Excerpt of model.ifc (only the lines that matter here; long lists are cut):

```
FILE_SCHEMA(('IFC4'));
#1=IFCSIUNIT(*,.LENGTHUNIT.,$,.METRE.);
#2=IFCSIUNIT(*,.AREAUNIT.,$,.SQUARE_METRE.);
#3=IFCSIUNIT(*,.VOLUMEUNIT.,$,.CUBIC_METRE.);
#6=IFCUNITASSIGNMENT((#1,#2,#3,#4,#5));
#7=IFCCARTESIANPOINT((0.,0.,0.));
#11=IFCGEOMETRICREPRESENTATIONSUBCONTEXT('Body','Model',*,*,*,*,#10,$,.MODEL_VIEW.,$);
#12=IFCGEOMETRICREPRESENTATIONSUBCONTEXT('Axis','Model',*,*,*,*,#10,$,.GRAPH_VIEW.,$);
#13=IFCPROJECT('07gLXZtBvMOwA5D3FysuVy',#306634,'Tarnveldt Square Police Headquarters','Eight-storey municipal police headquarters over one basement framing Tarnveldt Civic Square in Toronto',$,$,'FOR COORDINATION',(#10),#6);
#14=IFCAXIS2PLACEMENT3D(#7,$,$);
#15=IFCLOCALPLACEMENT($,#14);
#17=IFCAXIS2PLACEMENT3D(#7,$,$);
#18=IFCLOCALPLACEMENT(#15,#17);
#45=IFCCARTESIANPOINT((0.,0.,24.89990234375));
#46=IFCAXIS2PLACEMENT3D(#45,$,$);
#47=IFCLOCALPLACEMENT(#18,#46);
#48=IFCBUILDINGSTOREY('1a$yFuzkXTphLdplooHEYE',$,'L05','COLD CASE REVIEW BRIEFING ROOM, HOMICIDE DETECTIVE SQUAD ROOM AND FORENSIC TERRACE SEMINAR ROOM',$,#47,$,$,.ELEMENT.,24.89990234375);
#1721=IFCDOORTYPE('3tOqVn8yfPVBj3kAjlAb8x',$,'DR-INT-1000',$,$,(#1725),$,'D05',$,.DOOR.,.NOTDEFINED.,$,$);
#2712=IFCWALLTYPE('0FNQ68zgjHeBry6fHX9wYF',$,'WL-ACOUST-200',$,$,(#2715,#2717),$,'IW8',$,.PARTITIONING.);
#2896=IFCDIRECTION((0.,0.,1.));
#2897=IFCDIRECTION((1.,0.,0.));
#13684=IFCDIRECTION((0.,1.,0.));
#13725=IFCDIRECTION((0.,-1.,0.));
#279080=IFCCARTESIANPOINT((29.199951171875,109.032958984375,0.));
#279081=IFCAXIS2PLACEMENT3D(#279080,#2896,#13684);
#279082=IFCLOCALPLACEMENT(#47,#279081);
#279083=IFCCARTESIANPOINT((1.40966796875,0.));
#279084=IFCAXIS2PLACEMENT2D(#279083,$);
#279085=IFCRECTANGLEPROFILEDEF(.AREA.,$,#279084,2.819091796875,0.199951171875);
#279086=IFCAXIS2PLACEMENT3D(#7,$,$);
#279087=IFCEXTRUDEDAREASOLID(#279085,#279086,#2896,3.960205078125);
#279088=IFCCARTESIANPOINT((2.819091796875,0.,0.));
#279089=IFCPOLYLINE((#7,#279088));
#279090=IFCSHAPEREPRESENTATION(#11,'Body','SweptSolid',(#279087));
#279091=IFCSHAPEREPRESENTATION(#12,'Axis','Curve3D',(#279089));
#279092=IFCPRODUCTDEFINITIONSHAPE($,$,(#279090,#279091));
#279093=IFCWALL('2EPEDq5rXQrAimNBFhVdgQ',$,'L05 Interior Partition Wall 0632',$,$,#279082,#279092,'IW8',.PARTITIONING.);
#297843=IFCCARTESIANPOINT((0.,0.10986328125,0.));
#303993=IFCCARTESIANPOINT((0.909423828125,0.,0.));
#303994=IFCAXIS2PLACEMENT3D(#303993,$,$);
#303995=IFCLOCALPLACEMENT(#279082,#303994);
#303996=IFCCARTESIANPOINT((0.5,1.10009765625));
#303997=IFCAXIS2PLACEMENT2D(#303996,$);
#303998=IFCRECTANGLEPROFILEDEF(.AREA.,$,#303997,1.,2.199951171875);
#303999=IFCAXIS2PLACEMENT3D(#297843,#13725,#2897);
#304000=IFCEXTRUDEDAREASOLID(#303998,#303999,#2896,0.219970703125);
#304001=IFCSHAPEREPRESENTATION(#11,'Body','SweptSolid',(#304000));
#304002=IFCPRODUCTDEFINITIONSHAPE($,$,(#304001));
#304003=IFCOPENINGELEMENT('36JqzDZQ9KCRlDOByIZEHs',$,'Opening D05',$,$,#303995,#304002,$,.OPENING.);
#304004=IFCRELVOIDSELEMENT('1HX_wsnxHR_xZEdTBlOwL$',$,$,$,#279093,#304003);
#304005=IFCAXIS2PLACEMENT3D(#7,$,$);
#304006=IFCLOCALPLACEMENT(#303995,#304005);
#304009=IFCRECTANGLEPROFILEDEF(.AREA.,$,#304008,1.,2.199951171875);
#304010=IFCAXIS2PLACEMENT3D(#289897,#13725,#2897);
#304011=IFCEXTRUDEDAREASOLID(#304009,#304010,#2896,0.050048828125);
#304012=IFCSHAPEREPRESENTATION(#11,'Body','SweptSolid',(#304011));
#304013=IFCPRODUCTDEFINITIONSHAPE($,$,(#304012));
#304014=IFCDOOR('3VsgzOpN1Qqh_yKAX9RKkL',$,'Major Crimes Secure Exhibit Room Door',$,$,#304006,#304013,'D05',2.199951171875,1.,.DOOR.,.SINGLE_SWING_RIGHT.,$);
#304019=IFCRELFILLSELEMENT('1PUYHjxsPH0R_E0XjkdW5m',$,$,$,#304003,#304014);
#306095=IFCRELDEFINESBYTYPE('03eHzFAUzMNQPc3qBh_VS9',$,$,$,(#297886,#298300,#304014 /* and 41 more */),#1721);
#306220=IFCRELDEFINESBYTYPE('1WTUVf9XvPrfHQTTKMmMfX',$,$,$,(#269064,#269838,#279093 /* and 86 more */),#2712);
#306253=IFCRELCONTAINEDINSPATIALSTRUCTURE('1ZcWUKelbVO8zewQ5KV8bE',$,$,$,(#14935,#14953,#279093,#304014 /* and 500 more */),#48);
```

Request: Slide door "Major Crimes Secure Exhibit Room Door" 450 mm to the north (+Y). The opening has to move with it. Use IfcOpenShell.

```python
import ifcopenshell
import ifcopenshell.api.geometry
import ifcopenshell.util.placement
import ifcopenshell.util.unit

model = ifcopenshell.open("model.ifc")
unit_scale = ifcopenshell.util.unit.calculate_unit_scale(model)

door = model.by_id(304014)
opening = door.FillsVoids[0].RelatingOpeningElement
wall = opening.VoidsElements[0].RelatingBuildingElement

wall_matrix = ifcopenshell.util.placement.get_local_placement(wall.ObjectPlacement)
shift = wall_matrix[:3, 0] * 0.45 / unit_scale
before = ifcopenshell.util.placement.get_local_placement(door.ObjectPlacement)[:3, 3].copy()

# The door is placed relative to its opening, so it follows when the opening moves.
matrix = ifcopenshell.util.placement.get_local_placement(opening.ObjectPlacement)
matrix[:3, 3] += shift
ifcopenshell.api.geometry.edit_object_placement(
    model, product=opening, matrix=matrix, is_si=False, should_transform_children=True
)

after = ifcopenshell.util.placement.get_local_placement(door.ObjectPlacement)[:3, 3]
print("door moved by", (after - before).round(3) + 0.0)

model.write("model_rev.ifc")
```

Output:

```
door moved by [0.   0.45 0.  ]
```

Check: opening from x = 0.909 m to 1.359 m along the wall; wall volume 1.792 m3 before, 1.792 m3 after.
